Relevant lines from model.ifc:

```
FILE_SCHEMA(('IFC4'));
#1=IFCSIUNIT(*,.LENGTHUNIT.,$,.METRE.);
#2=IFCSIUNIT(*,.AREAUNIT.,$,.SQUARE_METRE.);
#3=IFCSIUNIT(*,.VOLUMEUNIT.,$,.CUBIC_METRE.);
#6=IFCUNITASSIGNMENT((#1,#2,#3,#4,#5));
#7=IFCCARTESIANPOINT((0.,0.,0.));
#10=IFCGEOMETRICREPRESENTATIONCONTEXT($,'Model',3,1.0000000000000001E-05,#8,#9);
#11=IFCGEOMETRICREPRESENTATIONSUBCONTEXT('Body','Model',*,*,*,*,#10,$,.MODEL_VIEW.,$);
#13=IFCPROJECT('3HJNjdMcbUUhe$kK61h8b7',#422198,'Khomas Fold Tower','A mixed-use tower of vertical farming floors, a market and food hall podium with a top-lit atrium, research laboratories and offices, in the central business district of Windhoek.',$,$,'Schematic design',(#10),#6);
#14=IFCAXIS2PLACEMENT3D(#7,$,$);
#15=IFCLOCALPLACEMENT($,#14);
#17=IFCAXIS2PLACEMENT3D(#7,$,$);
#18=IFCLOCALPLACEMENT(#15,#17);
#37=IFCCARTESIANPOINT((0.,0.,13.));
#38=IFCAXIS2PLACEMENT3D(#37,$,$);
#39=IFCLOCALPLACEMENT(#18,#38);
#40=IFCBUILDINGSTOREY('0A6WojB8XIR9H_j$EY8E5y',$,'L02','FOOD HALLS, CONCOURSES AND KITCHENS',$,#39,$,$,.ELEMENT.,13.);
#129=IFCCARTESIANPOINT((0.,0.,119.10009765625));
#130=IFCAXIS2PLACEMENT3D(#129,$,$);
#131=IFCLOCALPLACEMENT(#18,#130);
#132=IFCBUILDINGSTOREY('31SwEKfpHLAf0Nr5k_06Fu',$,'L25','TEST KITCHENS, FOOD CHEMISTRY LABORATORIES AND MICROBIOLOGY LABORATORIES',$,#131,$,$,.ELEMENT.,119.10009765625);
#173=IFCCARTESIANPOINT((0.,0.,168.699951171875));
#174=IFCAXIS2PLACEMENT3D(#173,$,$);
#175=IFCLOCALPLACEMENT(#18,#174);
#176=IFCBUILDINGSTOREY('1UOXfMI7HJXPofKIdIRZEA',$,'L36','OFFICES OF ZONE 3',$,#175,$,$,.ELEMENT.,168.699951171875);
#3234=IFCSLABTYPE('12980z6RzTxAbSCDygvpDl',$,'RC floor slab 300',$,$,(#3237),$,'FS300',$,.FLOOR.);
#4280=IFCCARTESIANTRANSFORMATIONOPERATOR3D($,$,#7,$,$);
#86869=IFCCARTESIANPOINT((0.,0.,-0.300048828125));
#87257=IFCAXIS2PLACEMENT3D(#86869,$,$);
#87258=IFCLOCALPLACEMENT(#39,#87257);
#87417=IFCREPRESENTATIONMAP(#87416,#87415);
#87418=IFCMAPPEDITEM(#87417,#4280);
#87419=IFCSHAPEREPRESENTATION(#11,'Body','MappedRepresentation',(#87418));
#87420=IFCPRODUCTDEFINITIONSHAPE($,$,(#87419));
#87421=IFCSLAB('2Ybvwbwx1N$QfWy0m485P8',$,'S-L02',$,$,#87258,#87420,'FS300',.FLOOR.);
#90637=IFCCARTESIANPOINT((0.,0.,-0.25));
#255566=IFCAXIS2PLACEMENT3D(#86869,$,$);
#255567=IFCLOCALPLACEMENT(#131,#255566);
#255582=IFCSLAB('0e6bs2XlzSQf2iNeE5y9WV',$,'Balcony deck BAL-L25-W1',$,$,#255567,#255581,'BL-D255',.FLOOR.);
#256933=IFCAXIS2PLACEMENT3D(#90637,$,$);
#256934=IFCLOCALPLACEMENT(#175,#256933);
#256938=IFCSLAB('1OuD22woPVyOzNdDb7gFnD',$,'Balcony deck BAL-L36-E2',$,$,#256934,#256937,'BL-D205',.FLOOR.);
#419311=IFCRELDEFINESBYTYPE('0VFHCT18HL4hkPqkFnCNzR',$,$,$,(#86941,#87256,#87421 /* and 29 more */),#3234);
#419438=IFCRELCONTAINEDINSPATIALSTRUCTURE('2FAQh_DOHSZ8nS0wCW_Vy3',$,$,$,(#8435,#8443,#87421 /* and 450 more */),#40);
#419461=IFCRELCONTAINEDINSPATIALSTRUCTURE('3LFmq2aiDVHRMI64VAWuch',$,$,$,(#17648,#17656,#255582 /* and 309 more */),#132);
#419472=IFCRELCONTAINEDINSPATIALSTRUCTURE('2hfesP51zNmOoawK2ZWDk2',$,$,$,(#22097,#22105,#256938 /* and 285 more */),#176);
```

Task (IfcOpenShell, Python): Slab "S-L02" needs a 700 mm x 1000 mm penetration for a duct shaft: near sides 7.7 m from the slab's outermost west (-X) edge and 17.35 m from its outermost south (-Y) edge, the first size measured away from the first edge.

```python
import numpy as np
import ifcopenshell
import ifcopenshell.api.feature
import ifcopenshell.api.geometry
import ifcopenshell.api.root
import ifcopenshell.geom
import ifcopenshell.util.placement
import ifcopenshell.util.representation
import ifcopenshell.util.shape
import ifcopenshell.util.unit

model = ifcopenshell.open("model.ifc")
unit_scale = ifcopenshell.util.unit.calculate_unit_scale(model)
settings = ifcopenshell.geom.settings()


def volume(element):
    """Net volume in cubic metres, openings subtracted."""
    shape = ifcopenshell.geom.create_shape(settings, element)
    return ifcopenshell.util.shape.get_volume(shape.geometry)


slab = model.by_guid("2Ybvwbwx1N$QfWy0m485P8")
before = volume(slab)

# Extent in the slab's own axes, in metres. The edges named are its -X and -Y sides.
slab_shape = ifcopenshell.geom.create_shape(settings, slab)
vertices = ifcopenshell.util.shape.get_vertices(slab_shape.geometry)
x_min, y_min, bottom = vertices.min(axis=0)
top = vertices[:, 2].max()

opening = ifcopenshell.api.root.create_entity(model, ifc_class="IfcOpeningElement", name="Duct shaft opening", predefined_type="OPENING")
context = ifcopenshell.util.representation.get_context(model, "Model", "Body", "MODEL_VIEW")
width, depth = 0.7, 1
outline = [(0.0, 0.0), (width, 0.0), (width, depth), (0.0, depth), (0.0, 0.0)]
# Overshoot both faces by 50 mm so the cut is clean.
shape = ifcopenshell.api.geometry.add_slab_representation(
    model, context=context, depth=top - bottom + 0.1, polyline=outline
)
ifcopenshell.api.geometry.assign_representation(model, product=opening, representation=shape)

matrix = ifcopenshell.util.placement.get_local_placement(slab.ObjectPlacement)
matrix[:, 3] = matrix @ np.append(np.array([x_min + 7.7, y_min + 17.35, bottom - 0.05]) / unit_scale, 1.0)
ifcopenshell.api.geometry.edit_object_placement(model, product=opening, matrix=matrix, is_si=False)
ifcopenshell.api.feature.add_feature(model, feature=opening, element=slab)

after = volume(slab)

print(f"slab volume {before:.3f} -> {after:.3f} m3")

model.write("model_rev.ifc")
```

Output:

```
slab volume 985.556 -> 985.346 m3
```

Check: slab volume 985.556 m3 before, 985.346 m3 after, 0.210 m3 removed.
